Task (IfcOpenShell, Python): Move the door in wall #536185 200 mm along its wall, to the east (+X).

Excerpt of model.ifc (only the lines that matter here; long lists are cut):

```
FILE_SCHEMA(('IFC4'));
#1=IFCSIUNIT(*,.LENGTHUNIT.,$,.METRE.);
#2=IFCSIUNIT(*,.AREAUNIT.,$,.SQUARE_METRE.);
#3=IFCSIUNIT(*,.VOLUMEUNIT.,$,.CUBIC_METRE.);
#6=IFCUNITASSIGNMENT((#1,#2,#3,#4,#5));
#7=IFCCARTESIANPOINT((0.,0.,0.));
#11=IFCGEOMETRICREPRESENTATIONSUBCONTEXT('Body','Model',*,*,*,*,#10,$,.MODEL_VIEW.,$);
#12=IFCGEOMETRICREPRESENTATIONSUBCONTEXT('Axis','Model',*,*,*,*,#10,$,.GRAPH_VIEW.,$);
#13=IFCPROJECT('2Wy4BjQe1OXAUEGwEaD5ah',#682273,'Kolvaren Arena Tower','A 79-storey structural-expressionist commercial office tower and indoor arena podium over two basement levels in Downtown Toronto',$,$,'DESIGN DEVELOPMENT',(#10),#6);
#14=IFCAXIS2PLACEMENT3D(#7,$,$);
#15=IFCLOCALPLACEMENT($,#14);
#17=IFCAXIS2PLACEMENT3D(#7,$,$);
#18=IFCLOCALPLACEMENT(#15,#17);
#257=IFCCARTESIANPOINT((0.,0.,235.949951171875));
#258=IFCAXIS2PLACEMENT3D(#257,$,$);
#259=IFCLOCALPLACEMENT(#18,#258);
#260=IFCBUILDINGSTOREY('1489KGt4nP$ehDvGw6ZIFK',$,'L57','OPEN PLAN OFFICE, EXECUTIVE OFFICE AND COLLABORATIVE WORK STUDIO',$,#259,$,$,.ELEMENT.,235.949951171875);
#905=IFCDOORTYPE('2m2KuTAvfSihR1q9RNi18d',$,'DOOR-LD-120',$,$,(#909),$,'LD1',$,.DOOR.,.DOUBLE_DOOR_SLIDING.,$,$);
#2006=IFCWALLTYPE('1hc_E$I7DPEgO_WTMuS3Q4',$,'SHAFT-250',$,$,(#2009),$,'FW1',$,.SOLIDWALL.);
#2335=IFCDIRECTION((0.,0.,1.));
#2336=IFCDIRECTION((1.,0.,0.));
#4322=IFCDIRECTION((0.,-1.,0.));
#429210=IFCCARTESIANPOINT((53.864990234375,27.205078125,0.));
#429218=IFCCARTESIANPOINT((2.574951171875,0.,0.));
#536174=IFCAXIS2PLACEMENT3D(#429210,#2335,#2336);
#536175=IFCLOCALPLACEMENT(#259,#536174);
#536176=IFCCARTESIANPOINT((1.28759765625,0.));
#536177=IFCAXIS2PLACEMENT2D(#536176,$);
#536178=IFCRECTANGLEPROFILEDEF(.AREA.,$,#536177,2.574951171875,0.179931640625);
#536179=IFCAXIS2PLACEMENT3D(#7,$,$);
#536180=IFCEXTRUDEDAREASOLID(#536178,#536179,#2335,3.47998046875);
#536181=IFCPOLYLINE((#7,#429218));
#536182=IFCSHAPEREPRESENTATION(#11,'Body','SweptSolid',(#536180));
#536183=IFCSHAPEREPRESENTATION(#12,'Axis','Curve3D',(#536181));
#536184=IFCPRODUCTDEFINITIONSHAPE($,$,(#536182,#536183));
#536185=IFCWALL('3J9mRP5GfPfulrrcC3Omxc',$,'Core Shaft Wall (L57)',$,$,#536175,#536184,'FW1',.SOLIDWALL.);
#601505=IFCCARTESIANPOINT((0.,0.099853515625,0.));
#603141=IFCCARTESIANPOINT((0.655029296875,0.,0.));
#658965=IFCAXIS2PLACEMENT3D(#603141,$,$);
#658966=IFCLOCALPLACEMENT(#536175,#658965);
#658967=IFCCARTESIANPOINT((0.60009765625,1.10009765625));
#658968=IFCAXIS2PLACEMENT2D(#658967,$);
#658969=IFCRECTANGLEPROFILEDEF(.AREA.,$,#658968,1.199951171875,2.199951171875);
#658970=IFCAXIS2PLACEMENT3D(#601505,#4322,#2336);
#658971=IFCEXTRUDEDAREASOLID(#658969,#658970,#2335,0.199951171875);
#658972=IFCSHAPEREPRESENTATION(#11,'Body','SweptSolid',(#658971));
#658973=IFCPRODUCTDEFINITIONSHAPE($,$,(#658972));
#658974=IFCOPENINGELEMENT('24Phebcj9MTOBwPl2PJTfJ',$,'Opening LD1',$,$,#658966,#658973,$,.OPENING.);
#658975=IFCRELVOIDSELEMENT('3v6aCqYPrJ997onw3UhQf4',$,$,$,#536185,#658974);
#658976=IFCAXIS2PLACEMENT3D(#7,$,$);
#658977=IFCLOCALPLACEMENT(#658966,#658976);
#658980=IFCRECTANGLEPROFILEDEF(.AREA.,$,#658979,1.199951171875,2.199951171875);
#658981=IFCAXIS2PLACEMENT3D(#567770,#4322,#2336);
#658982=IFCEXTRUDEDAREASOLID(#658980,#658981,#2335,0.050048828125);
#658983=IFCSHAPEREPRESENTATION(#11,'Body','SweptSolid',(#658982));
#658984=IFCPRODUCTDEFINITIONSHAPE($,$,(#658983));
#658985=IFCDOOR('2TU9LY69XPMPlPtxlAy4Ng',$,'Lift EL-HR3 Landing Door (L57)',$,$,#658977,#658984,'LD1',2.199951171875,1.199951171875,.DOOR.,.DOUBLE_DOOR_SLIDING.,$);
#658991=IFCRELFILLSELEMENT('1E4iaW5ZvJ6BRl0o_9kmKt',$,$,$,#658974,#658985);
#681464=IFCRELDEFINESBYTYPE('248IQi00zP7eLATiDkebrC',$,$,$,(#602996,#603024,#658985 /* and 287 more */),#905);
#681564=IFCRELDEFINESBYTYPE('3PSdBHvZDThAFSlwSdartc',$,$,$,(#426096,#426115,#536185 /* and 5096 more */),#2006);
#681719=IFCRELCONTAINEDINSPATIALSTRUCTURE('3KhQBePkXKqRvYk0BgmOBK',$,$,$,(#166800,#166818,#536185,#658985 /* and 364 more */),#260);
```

```python
import ifcopenshell
import ifcopenshell.api.geometry
import ifcopenshell.util.placement

model = ifcopenshell.open("model.ifc")

door = model.by_guid("2TU9LY69XPMPlPtxlAy4Ng")
opening = door.FillsVoids[0].RelatingOpeningElement
wall = opening.VoidsElements[0].RelatingBuildingElement

wall_matrix = ifcopenshell.util.placement.get_local_placement(wall.ObjectPlacement)
shift = wall_matrix[:3, 0] * 0.2
before = ifcopenshell.util.placement.get_local_placement(door.ObjectPlacement)[:3, 3].copy()

# The door is placed relative to its opening, so it follows when the opening moves.
matrix = ifcopenshell.util.placement.get_local_placement(opening.ObjectPlacement)
matrix[:3, 3] += shift
ifcopenshell.api.geometry.edit_object_placement(
    model, product=opening, matrix=matrix, is_si=False, should_transform_children=True
)

after = ifcopenshell.util.placement.get_local_placement(door.ObjectPlacement)[:3, 3]
print("door moved by", (after - before).round(3) + 0.0)

model.write("model_edited.ifc")
```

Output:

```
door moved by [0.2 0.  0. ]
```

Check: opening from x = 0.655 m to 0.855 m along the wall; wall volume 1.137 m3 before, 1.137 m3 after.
